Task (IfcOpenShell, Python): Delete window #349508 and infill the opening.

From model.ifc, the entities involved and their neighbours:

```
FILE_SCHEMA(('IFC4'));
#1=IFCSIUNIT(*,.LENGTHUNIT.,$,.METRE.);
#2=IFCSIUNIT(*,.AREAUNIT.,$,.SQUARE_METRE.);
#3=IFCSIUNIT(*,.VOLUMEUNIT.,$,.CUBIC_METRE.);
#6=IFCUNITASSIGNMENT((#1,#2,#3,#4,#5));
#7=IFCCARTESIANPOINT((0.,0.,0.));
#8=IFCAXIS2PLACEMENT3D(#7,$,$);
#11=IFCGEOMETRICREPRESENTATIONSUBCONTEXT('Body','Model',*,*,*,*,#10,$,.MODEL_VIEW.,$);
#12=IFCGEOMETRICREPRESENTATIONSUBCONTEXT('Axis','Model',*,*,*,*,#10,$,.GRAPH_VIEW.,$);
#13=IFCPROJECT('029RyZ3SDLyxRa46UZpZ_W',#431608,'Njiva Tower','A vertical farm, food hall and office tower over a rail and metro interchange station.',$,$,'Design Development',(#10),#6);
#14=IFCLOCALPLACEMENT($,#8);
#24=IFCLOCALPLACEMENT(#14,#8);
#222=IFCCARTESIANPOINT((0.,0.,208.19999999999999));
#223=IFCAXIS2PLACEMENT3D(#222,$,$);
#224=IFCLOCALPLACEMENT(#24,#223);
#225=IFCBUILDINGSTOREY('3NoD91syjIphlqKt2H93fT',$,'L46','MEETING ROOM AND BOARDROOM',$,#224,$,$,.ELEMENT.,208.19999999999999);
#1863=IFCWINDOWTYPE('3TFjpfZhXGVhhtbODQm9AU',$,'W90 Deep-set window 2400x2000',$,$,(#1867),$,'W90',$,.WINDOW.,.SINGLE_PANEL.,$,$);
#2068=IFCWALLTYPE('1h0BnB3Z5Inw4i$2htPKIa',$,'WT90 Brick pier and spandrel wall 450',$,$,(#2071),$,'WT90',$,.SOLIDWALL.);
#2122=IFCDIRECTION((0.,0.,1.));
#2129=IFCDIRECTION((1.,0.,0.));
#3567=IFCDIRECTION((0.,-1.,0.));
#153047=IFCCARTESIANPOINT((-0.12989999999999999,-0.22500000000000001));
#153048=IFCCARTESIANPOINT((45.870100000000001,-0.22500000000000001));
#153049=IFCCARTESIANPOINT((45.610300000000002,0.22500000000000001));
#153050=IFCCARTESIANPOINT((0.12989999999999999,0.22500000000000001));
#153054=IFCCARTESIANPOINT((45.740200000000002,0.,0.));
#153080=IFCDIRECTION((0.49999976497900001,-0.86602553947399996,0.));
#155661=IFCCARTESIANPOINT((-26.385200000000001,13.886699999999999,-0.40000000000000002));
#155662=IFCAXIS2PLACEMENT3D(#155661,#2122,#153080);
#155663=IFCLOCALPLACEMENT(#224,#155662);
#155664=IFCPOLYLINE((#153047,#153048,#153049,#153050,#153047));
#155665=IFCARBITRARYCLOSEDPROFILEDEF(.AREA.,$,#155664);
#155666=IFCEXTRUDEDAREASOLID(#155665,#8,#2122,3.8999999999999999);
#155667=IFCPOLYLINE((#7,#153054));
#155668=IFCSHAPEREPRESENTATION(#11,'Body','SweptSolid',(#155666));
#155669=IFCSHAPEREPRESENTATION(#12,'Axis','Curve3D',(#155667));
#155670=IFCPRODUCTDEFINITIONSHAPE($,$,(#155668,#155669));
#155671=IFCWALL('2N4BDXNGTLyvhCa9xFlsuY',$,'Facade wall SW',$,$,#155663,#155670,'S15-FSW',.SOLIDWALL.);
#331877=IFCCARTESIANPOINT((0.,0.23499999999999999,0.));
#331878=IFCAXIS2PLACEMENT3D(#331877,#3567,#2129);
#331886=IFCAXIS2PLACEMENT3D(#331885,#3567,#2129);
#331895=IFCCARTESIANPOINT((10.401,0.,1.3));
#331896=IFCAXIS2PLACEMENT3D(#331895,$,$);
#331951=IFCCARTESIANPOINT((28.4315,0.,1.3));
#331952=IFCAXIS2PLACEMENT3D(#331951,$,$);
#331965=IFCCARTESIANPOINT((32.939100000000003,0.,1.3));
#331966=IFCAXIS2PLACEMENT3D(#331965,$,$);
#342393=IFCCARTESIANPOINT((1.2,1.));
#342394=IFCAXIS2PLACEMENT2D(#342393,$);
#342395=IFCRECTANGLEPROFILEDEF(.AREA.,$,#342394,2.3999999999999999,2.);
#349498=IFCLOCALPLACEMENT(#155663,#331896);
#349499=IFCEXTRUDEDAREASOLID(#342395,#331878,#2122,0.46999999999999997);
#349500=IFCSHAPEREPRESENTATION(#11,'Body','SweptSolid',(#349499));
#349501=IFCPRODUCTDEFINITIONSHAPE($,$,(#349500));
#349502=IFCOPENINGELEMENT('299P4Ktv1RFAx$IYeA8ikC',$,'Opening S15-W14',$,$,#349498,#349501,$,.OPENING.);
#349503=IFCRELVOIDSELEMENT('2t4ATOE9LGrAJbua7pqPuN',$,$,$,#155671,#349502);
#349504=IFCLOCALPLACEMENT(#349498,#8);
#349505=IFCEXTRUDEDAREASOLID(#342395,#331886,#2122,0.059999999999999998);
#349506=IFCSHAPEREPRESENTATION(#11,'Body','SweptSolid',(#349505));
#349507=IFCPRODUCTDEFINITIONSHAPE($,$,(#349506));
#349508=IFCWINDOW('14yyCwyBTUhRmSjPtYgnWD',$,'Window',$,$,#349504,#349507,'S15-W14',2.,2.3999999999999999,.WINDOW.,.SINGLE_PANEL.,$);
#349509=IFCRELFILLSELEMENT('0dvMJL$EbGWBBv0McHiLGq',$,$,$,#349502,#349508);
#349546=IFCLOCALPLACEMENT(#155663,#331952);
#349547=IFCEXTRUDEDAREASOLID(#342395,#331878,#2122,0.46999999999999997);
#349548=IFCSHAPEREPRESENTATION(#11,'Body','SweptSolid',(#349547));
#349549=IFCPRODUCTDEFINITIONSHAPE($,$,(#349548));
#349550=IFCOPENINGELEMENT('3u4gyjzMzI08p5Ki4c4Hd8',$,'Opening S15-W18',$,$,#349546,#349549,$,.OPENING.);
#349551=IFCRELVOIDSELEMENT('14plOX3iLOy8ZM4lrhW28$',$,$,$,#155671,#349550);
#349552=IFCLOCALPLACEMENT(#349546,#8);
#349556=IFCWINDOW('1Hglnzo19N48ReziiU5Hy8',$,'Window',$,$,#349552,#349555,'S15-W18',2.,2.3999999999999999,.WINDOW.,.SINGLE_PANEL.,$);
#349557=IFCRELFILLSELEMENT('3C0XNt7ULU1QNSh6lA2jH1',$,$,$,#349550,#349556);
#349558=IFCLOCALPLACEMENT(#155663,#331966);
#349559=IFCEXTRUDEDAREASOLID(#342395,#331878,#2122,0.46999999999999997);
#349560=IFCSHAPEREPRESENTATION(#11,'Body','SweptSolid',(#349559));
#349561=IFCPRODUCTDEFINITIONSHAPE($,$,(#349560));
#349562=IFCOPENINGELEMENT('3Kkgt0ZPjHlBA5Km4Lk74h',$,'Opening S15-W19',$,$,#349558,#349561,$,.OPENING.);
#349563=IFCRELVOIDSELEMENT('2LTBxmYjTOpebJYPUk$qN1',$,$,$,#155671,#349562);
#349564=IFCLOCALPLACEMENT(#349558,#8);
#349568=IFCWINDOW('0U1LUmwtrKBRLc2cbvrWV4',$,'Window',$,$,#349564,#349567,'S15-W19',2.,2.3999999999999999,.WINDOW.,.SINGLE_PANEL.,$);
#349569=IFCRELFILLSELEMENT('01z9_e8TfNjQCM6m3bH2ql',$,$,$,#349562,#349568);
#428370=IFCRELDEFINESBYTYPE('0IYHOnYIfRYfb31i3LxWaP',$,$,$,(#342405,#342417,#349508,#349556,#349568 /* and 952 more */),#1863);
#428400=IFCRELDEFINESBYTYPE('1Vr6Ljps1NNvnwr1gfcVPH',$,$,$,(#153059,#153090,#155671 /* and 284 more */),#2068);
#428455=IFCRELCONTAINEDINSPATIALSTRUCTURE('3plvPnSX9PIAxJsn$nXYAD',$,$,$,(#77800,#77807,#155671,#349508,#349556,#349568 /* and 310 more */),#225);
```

```python
import ifcopenshell
import ifcopenshell.api.feature
import ifcopenshell.api.root
import ifcopenshell.geom
import ifcopenshell.util.shape

model = ifcopenshell.open("model.ifc")
settings = ifcopenshell.geom.settings()


def volume(element):
    """Net volume in cubic metres, openings subtracted."""
    shape = ifcopenshell.geom.create_shape(settings, element)
    return ifcopenshell.util.shape.get_volume(shape.geometry)


window = model.by_id(349508)
opening = window.FillsVoids[0].RelatingOpeningElement
wall = opening.VoidsElements[0].RelatingBuildingElement
before = volume(wall)

ifcopenshell.api.root.remove_product(model, product=window)
ifcopenshell.api.feature.remove_feature(model, feature=opening)

after = volume(wall)

print(f"wall volume {before:.3f} -> {after:.3f} m3")

model.write("model_rev.ifc")
```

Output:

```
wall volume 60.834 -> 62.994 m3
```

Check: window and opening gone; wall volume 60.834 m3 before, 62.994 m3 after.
